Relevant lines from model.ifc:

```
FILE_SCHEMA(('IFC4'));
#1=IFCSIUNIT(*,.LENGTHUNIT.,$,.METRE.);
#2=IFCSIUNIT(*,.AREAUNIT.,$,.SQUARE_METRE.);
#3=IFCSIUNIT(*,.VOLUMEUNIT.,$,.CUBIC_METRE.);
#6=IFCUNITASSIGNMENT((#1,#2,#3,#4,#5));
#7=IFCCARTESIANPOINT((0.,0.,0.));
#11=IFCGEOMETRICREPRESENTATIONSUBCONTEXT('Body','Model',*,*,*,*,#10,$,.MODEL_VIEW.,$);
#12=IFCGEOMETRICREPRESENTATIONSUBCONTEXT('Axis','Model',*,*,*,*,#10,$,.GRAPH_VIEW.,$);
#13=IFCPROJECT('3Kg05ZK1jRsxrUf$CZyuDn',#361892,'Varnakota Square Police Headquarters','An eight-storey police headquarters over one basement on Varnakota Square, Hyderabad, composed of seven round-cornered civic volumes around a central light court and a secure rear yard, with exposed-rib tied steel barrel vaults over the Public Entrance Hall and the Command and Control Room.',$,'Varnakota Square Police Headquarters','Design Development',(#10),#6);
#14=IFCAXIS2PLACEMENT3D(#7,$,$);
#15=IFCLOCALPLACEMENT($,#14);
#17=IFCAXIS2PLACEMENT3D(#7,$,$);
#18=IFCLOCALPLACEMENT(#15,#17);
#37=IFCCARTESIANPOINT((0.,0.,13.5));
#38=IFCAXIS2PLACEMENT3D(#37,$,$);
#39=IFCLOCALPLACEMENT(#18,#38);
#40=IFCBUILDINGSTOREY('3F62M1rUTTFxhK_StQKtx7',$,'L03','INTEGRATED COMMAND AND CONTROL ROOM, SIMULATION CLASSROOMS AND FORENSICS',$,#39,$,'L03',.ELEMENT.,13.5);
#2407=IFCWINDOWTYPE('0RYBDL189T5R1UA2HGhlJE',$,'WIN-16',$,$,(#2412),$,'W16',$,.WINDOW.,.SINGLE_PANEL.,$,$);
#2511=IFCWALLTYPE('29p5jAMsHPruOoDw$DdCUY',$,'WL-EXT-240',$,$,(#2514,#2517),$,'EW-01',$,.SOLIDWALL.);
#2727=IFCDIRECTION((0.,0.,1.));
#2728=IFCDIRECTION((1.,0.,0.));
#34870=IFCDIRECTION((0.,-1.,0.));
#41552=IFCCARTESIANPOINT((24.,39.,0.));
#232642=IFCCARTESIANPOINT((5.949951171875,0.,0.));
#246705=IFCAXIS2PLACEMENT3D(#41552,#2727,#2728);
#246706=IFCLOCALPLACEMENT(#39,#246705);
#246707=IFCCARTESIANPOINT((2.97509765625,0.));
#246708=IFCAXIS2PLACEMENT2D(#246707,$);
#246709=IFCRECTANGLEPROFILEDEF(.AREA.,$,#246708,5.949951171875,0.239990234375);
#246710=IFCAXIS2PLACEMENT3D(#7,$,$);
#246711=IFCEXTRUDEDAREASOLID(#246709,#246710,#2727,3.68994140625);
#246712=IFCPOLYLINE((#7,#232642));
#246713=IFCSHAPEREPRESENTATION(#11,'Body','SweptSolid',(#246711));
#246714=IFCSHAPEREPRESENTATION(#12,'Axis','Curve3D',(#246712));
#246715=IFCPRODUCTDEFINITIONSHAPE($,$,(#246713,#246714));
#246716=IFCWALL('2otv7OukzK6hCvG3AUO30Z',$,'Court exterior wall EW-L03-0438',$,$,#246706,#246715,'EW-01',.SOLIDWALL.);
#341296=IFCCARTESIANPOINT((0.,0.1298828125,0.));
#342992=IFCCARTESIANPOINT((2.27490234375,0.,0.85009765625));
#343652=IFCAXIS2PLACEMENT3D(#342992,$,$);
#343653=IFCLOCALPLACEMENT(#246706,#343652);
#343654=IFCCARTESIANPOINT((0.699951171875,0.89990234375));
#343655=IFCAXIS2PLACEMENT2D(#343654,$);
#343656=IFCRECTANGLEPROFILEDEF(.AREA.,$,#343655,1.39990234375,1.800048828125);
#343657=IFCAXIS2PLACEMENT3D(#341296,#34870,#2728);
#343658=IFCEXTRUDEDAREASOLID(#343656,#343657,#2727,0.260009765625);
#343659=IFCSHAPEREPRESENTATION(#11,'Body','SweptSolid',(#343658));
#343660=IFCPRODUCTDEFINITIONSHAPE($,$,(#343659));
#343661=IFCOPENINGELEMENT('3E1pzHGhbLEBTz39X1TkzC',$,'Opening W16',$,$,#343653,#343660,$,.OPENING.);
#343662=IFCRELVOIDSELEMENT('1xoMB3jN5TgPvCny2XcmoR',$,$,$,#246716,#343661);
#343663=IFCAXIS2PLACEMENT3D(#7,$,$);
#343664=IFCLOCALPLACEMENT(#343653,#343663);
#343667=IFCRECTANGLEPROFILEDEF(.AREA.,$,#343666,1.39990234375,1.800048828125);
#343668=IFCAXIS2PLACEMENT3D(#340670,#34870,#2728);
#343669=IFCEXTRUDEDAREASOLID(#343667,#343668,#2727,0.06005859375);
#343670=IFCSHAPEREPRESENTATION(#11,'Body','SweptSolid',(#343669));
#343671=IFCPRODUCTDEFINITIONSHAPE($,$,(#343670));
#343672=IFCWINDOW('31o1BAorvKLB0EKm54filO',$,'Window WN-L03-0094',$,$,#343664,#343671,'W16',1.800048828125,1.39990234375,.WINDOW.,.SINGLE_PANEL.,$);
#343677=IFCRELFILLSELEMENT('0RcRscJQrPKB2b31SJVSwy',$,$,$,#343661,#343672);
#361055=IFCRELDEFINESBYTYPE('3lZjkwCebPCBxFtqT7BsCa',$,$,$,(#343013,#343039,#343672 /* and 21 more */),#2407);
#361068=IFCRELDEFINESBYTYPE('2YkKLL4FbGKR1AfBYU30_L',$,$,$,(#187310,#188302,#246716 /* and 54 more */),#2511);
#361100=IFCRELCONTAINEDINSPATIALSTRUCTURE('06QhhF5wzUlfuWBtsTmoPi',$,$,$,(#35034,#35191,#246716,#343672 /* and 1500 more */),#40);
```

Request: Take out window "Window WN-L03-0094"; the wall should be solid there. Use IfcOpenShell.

```python
import ifcopenshell
import ifcopenshell.api.feature
import ifcopenshell.api.root
import ifcopenshell.geom
import ifcopenshell.util.shape

model = ifcopenshell.open("model.ifc")
settings = ifcopenshell.geom.settings()


def volume(element):
    """Net volume in cubic metres, openings subtracted."""
    shape = ifcopenshell.geom.create_shape(settings, element)
    return ifcopenshell.util.shape.get_volume(shape.geometry)


window = model.by_id(343672)
opening = window.FillsVoids[0].RelatingOpeningElement
wall = opening.VoidsElements[0].RelatingBuildingElement
before = volume(wall)

ifcopenshell.api.root.remove_product(model, product=window)
ifcopenshell.api.feature.remove_feature(model, feature=opening)

after = volume(wall)

print(f"wall volume {before:.3f} -> {after:.3f} m3")

model.write("model-out.ifc")
```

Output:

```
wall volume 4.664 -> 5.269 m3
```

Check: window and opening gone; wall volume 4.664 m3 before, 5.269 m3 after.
